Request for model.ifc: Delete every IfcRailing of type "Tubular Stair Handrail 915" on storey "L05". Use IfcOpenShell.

First a look at what the model holds.

```python
import ifcopenshell
import ifcopenshell.util.element

model = ifcopenshell.open("model.ifc")
print(model.schema)
storey = next(s for s in model.by_type("IfcBuildingStorey") if s.Name == "L05")
railings = [e for e in ifcopenshell.util.element.get_decomposition(storey) if e.is_a("IfcRailing")]
seen = {}
for e in railings:
    element_type = ifcopenshell.util.element.get_type(e)
    name = element_type.Name if element_type not in (None, e) else None
    seen[name] = seen.get(name, 0) + 1
for name, count in sorted(seen.items(), key=str):
    print(count, "x", name)
```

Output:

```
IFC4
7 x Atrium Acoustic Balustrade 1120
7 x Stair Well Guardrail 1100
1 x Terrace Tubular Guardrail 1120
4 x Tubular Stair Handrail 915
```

```python
import ifcopenshell
import ifcopenshell.api.root
import ifcopenshell.util.element

model = ifcopenshell.open("model.ifc")

storey = next(s for s in model.by_type("IfcBuildingStorey") if s.Name == "L05")
railings = [e for e in ifcopenshell.util.element.get_decomposition(storey) if e.is_a("IfcRailing")]
targets = [e for e in railings if (t := ifcopenshell.util.element.get_type(e)) not in (None, e) and t.Name == "Tubular Stair Handrail 915"]

for e in targets:
    ifcopenshell.api.root.remove_product(model, product=e)
print(len(targets), "removed")

model.write("model_rev.ifc")
```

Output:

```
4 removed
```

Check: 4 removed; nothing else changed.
